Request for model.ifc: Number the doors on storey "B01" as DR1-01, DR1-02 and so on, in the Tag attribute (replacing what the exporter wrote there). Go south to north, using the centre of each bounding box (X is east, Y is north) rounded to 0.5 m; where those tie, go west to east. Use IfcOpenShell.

First a look at what the model holds.

```python
import ifcopenshell
import ifcopenshell.util.element
import ifcopenshell.util.placement

model = ifcopenshell.open("model.ifc")
print(model.schema)
storey = next(s for s in model.by_type("IfcBuildingStorey") if s.Name == "B01")
doors = [e for e in ifcopenshell.util.element.get_decomposition(storey) if e.is_a("IfcDoor")]
for e in sorted(doors, key=lambda e: e.id()):
    origin = ifcopenshell.util.placement.get_local_placement(e.ObjectPlacement)[:3, 3]
    print(e.id(), e.Tag, e.Name, origin.round(2) + 0.0, sep=" | ")
```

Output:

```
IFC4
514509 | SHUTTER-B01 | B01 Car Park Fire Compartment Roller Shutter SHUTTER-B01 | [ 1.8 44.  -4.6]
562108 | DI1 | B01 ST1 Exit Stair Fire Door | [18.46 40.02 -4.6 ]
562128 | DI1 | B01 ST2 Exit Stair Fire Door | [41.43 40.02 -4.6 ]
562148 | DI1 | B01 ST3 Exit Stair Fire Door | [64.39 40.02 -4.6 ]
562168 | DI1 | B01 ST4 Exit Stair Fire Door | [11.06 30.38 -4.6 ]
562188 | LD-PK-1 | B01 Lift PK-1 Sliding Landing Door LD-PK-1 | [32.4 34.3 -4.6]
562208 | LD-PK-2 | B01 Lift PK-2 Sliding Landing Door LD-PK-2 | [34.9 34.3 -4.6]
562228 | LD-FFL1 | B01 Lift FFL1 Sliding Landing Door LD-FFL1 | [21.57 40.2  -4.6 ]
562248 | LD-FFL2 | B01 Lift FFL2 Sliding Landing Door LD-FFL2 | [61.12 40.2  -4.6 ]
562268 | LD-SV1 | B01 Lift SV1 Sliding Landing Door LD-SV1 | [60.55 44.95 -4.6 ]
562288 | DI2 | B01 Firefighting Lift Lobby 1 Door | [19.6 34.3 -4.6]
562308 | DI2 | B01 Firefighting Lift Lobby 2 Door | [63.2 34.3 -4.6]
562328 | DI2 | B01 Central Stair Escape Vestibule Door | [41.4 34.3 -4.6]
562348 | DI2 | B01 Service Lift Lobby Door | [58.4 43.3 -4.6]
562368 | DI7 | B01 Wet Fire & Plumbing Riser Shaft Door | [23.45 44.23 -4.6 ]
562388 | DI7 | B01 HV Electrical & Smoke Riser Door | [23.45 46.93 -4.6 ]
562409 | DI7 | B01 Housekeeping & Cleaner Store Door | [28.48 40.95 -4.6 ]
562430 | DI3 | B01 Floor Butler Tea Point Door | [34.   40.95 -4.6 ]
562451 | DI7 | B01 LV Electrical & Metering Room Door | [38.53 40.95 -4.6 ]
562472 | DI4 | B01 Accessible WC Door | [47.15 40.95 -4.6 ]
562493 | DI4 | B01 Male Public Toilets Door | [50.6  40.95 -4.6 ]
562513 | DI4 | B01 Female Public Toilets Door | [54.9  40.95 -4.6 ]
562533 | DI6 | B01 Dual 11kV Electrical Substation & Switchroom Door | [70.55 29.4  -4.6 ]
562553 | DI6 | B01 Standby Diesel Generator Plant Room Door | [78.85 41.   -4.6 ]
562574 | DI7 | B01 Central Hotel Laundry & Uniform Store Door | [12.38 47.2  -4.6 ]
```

```python
import ifcopenshell
import ifcopenshell.geom
import ifcopenshell.util.element
import ifcopenshell.util.shape

model = ifcopenshell.open("model.ifc")
settings = ifcopenshell.geom.settings()
settings.set("use-world-coords", True)


def centre(element):
    shape = ifcopenshell.geom.create_shape(settings, element)
    return ifcopenshell.util.shape.get_bbox_centroid(shape.geometry)


storey = next(s for s in model.by_type("IfcBuildingStorey") if s.Name == "B01")
doors = [e for e in ifcopenshell.util.element.get_decomposition(storey) if e.is_a("IfcDoor")]

# Insertion points can sit at a corner or the storey origin, so sort by the geometry (in metres).
centres = {e: centre(e) for e in doors}
doors.sort(key=lambda e: (round(centres[e][1] / 0.5), centres[e][0]))

for i, e in enumerate(doors, start=1):
    number = f"DR1-{i:02d}"
    e.Tag = number
    print(e.id(), number)

model.write("model_rev.ifc")
```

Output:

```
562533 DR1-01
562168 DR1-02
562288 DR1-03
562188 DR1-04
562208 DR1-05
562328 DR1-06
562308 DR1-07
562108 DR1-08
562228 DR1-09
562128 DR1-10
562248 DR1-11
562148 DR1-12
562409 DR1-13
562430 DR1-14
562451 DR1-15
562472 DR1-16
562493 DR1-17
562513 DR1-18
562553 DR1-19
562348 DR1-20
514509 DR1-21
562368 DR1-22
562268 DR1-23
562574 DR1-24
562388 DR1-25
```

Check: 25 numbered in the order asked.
